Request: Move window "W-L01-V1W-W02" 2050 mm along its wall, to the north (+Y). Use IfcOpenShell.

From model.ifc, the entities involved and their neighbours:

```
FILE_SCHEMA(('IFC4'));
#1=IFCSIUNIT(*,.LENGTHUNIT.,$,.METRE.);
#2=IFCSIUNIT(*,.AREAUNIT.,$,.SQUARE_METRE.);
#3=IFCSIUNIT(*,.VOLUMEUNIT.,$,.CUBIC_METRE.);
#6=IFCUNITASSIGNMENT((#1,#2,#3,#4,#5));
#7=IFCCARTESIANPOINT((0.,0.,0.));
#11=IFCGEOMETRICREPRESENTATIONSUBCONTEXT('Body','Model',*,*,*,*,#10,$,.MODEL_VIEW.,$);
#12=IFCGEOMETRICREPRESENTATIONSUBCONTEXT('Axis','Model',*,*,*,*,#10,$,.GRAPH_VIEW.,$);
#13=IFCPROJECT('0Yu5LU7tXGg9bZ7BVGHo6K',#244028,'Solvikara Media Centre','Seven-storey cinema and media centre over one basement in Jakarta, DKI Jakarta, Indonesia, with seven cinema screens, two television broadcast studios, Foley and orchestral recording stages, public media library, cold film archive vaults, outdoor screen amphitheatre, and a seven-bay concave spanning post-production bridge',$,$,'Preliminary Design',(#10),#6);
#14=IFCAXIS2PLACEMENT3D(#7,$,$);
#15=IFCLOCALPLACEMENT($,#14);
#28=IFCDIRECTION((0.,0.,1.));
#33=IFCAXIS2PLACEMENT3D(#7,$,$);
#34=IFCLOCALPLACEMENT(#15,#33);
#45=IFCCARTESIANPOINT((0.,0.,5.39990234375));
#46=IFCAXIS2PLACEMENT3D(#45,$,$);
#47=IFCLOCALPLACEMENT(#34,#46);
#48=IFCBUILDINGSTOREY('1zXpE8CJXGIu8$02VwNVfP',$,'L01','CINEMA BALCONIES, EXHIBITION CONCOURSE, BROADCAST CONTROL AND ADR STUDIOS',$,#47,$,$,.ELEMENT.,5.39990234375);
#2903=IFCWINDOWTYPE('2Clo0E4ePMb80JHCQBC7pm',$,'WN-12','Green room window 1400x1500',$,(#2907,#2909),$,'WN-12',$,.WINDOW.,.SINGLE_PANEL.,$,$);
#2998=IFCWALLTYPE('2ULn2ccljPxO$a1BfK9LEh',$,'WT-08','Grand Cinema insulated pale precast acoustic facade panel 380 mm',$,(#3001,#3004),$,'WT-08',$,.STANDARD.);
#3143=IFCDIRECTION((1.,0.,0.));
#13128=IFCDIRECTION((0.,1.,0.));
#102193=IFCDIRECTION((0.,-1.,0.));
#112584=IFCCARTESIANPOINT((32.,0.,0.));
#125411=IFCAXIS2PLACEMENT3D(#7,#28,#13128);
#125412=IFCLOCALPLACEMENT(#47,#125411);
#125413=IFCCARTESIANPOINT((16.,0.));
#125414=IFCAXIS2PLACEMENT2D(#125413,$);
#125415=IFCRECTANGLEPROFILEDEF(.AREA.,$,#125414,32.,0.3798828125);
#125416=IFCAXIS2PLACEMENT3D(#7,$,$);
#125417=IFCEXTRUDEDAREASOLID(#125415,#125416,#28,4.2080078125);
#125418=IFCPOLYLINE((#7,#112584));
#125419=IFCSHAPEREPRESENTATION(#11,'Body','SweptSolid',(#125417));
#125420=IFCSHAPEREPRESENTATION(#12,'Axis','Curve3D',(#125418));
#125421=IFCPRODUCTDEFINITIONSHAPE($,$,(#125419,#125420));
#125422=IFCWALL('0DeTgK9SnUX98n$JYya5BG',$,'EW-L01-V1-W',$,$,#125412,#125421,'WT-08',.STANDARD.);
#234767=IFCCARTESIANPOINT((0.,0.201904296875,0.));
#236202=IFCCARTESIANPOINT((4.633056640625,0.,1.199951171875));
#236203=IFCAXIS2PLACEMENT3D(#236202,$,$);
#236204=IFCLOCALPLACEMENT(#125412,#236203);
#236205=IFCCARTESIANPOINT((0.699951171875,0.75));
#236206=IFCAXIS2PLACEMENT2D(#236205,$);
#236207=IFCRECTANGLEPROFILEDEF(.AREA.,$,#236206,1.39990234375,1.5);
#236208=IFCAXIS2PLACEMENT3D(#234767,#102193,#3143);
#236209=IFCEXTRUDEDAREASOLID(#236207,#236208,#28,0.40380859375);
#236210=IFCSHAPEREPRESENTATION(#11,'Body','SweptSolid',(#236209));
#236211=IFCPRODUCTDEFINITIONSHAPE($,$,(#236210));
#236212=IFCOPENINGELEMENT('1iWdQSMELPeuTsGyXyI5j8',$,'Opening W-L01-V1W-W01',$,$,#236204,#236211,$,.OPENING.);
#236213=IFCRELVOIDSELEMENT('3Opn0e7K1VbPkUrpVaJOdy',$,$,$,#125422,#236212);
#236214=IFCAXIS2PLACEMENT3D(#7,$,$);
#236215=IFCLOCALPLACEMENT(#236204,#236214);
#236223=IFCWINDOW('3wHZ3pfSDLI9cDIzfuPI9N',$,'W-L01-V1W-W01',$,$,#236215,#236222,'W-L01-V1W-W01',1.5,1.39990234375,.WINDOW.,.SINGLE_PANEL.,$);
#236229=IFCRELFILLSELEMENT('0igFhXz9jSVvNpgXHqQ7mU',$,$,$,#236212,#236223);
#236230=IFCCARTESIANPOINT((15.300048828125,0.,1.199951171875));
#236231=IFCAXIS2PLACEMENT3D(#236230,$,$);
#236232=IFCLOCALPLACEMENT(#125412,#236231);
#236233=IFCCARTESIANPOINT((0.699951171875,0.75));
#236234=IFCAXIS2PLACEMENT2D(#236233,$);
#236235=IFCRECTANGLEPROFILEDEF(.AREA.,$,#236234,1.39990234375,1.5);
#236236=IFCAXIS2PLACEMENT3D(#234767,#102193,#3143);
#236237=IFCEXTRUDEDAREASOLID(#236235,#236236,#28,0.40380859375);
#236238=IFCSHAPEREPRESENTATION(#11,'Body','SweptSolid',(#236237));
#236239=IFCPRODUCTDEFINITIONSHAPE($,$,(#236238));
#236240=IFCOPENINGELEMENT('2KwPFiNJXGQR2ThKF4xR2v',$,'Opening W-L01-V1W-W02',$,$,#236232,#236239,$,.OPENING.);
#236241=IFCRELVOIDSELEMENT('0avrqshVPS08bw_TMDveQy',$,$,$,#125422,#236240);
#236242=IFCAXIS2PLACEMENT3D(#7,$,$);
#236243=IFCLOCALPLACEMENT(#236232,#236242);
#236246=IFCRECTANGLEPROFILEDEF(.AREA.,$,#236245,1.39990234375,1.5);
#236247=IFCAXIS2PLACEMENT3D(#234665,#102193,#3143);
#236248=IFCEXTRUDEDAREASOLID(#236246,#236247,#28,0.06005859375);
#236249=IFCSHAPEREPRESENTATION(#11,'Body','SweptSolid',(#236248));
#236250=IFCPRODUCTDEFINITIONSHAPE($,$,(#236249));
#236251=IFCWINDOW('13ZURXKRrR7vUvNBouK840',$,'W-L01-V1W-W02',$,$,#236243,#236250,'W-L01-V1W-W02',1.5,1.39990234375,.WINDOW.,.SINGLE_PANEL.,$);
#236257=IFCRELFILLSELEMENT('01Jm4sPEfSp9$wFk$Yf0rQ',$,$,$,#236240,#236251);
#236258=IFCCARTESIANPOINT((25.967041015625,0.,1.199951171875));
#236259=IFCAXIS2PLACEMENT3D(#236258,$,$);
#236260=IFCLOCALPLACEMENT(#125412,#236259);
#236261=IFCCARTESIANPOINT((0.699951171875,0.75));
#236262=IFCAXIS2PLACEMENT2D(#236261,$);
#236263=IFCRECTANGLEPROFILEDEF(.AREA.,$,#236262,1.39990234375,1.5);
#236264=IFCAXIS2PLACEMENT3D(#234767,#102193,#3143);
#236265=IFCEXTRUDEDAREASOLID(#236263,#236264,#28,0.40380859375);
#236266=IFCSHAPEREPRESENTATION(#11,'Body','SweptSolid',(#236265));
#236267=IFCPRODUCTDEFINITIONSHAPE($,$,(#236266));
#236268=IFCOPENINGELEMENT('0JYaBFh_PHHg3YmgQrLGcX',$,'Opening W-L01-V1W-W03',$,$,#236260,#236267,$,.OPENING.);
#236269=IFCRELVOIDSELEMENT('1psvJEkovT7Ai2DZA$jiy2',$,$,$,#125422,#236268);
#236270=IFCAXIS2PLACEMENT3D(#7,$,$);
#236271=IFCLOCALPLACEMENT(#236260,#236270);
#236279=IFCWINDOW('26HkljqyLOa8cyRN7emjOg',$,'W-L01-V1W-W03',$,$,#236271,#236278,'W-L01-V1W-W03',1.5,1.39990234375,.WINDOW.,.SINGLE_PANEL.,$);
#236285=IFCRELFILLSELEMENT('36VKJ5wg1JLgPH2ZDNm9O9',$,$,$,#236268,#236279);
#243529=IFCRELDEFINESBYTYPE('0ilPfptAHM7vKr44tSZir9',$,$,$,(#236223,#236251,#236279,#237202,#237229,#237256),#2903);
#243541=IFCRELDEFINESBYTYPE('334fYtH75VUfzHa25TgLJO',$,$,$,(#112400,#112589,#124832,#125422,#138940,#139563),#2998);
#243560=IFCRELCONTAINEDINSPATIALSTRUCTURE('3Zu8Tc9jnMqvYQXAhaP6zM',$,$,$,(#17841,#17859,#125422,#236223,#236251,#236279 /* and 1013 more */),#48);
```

```python
import ifcopenshell
import ifcopenshell.api.geometry
import ifcopenshell.util.placement
import ifcopenshell.util.unit

model = ifcopenshell.open("model.ifc")
unit_scale = ifcopenshell.util.unit.calculate_unit_scale(model)

window = model.by_guid("13ZURXKRrR7vUvNBouK840")
opening = window.FillsVoids[0].RelatingOpeningElement
wall = opening.VoidsElements[0].RelatingBuildingElement

wall_matrix = ifcopenshell.util.placement.get_local_placement(wall.ObjectPlacement)
shift = wall_matrix[:3, 0] * 2.05 / unit_scale
before = ifcopenshell.util.placement.get_local_placement(window.ObjectPlacement)[:3, 3].copy()

# The window is placed relative to its opening, so it follows when the opening moves.
matrix = ifcopenshell.util.placement.get_local_placement(opening.ObjectPlacement)
matrix[:3, 3] += shift
ifcopenshell.api.geometry.edit_object_placement(
    model, product=opening, matrix=matrix, is_si=False, should_transform_children=True
)

after = ifcopenshell.util.placement.get_local_placement(window.ObjectPlacement)[:3, 3]
print("window moved by", (after - before).round(3) + 0.0)

model.write("model_updated.ifc")
```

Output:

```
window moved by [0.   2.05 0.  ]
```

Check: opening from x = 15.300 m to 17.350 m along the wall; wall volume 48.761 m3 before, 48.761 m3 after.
